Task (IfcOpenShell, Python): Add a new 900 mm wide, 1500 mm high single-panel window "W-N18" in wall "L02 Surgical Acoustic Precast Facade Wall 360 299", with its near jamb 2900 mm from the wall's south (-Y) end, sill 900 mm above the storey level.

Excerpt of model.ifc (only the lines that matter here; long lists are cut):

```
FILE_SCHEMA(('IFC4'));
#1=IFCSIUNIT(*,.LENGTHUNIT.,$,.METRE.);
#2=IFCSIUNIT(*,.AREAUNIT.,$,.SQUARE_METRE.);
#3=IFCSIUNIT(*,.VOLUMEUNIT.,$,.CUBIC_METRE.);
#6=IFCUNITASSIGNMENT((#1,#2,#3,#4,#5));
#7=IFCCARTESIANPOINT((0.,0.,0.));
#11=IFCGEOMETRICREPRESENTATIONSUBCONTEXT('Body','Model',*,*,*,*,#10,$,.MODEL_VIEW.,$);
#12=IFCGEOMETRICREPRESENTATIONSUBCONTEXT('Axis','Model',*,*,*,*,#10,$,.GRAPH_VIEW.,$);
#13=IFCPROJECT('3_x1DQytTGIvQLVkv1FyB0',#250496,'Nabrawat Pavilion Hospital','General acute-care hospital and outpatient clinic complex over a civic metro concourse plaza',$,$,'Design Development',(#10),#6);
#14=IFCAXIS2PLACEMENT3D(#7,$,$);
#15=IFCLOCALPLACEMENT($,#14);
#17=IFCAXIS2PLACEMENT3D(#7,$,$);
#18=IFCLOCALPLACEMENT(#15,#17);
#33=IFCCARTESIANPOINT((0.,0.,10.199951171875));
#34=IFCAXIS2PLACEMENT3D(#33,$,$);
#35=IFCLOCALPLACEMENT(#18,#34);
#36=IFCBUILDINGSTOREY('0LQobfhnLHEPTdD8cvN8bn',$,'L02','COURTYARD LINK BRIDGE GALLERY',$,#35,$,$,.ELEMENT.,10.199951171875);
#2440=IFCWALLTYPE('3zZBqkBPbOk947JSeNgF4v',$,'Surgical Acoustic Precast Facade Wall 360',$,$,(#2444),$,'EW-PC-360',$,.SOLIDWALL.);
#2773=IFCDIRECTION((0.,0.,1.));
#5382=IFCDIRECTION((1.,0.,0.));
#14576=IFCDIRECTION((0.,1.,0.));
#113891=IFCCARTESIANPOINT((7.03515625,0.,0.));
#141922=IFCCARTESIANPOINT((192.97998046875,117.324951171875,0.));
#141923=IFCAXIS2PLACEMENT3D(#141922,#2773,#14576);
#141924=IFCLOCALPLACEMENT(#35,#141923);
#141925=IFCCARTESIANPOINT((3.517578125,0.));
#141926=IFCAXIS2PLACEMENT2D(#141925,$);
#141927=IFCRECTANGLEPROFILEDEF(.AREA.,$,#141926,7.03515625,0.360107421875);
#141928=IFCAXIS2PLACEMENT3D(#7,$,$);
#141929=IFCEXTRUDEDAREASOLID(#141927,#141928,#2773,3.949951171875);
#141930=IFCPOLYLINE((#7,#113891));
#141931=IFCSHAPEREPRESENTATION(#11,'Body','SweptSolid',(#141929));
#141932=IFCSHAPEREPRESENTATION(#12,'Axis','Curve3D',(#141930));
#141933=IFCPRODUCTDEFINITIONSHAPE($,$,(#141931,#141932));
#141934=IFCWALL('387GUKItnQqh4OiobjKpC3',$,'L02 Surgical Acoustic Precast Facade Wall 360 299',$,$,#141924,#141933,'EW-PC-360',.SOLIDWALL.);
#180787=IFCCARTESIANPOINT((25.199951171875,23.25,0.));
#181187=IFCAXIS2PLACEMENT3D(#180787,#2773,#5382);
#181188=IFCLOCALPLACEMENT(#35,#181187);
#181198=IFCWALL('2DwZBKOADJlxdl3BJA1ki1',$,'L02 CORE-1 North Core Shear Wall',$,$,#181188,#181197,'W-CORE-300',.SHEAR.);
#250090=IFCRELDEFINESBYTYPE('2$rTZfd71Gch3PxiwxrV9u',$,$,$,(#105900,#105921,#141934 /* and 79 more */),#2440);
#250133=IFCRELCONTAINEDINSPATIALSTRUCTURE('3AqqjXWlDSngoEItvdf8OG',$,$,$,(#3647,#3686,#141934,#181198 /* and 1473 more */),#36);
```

```python
import numpy as np
import ifcopenshell
import ifcopenshell.api.feature
import ifcopenshell.api.geometry
import ifcopenshell.api.root
import ifcopenshell.api.spatial
import ifcopenshell.geom
import ifcopenshell.util.element
import ifcopenshell.util.placement
import ifcopenshell.util.representation
import ifcopenshell.util.shape
import ifcopenshell.util.unit

model = ifcopenshell.open("model.ifc")
unit_scale = ifcopenshell.util.unit.calculate_unit_scale(model)
settings = ifcopenshell.geom.settings()


def volume(element):
    """Net volume in cubic metres, openings subtracted."""
    shape = ifcopenshell.geom.create_shape(settings, element)
    return ifcopenshell.util.shape.get_volume(shape.geometry)


wall = model.by_guid("387GUKItnQqh4OiobjKpC3")
storey = ifcopenshell.util.element.get_container(wall, ifc_class="IfcBuildingStorey")
context = ifcopenshell.util.representation.get_context(model, "Model", "Body", "MODEL_VIEW")
before = volume(wall)

width, height, from_end, sill = 0.9, 1.5, 2.9, 0.9  # metres

# The wall runs along its own X axis, and the end named is its -X end.
wall_shape = ifcopenshell.geom.create_shape(settings, wall)
x, y, z = ifcopenshell.util.shape.get_vertices(wall_shape.geometry).T
start = x.min() + from_end
face, thickness = float(y.min()), float(y.max() - y.min())
wall_matrix = ifcopenshell.util.placement.get_local_placement(wall.ObjectPlacement)
level = ifcopenshell.util.placement.get_local_placement(storey.ObjectPlacement)[2, 3]


def in_wall(x, y):
    """Placement at x, y metres in the wall's axes, at sill height."""
    matrix = wall_matrix.copy()
    matrix[:, 3] = wall_matrix @ np.array([x / unit_scale, y / unit_scale, 0.0, 1.0])
    matrix[2, 3] = level + sill / unit_scale
    return matrix


# Opening: a box that overshoots both wall faces by 50 mm.
opening = ifcopenshell.api.root.create_entity(model, ifc_class="IfcOpeningElement", predefined_type="OPENING")
box = ifcopenshell.api.geometry.add_wall_representation(
    model, context=context, length=width, height=height, thickness=thickness + 0.1
)
ifcopenshell.api.geometry.assign_representation(model, product=opening, representation=box)
ifcopenshell.api.geometry.edit_object_placement(model, product=opening, matrix=in_wall(start, face - 0.05), is_si=False)
ifcopenshell.api.feature.add_feature(model, feature=opening, element=wall)

window = ifcopenshell.api.root.create_entity(model, ifc_class="IfcWindow", name="W-N18", predefined_type="WINDOW")
window.OverallWidth, window.OverallHeight = width / unit_scale, height / unit_scale
window.PartitioningType = "SINGLE_PANEL"
body = ifcopenshell.api.geometry.add_window_representation(
    model,
    context=context,
    overall_width=window.OverallWidth,
    overall_height=window.OverallHeight,
    partition_type="SINGLE_PANEL",
)
ifcopenshell.api.geometry.assign_representation(model, product=window, representation=body)
ifcopenshell.api.spatial.assign_container(model, products=[window], relating_structure=storey)
ifcopenshell.api.feature.add_filling(model, opening=opening, element=window)

# Centre the window in the wall's thickness.
ifcopenshell.api.geometry.edit_object_placement(model, product=window, matrix=in_wall(start, face), is_si=False)
window_shape = ifcopenshell.geom.create_shape(settings, window)
depth = ifcopenshell.util.shape.get_vertices(window_shape.geometry)[:, 1]
offset = face + thickness / 2 - (depth.min() + depth.max()) / 2
ifcopenshell.api.geometry.edit_object_placement(model, product=window, matrix=in_wall(start, offset), is_si=False)

after = volume(wall)

print(f"wall volume {before:.3f} -> {after:.3f} m3")

model.write("model_updated.ifc")
```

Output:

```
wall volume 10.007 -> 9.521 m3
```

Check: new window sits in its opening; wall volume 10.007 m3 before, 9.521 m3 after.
